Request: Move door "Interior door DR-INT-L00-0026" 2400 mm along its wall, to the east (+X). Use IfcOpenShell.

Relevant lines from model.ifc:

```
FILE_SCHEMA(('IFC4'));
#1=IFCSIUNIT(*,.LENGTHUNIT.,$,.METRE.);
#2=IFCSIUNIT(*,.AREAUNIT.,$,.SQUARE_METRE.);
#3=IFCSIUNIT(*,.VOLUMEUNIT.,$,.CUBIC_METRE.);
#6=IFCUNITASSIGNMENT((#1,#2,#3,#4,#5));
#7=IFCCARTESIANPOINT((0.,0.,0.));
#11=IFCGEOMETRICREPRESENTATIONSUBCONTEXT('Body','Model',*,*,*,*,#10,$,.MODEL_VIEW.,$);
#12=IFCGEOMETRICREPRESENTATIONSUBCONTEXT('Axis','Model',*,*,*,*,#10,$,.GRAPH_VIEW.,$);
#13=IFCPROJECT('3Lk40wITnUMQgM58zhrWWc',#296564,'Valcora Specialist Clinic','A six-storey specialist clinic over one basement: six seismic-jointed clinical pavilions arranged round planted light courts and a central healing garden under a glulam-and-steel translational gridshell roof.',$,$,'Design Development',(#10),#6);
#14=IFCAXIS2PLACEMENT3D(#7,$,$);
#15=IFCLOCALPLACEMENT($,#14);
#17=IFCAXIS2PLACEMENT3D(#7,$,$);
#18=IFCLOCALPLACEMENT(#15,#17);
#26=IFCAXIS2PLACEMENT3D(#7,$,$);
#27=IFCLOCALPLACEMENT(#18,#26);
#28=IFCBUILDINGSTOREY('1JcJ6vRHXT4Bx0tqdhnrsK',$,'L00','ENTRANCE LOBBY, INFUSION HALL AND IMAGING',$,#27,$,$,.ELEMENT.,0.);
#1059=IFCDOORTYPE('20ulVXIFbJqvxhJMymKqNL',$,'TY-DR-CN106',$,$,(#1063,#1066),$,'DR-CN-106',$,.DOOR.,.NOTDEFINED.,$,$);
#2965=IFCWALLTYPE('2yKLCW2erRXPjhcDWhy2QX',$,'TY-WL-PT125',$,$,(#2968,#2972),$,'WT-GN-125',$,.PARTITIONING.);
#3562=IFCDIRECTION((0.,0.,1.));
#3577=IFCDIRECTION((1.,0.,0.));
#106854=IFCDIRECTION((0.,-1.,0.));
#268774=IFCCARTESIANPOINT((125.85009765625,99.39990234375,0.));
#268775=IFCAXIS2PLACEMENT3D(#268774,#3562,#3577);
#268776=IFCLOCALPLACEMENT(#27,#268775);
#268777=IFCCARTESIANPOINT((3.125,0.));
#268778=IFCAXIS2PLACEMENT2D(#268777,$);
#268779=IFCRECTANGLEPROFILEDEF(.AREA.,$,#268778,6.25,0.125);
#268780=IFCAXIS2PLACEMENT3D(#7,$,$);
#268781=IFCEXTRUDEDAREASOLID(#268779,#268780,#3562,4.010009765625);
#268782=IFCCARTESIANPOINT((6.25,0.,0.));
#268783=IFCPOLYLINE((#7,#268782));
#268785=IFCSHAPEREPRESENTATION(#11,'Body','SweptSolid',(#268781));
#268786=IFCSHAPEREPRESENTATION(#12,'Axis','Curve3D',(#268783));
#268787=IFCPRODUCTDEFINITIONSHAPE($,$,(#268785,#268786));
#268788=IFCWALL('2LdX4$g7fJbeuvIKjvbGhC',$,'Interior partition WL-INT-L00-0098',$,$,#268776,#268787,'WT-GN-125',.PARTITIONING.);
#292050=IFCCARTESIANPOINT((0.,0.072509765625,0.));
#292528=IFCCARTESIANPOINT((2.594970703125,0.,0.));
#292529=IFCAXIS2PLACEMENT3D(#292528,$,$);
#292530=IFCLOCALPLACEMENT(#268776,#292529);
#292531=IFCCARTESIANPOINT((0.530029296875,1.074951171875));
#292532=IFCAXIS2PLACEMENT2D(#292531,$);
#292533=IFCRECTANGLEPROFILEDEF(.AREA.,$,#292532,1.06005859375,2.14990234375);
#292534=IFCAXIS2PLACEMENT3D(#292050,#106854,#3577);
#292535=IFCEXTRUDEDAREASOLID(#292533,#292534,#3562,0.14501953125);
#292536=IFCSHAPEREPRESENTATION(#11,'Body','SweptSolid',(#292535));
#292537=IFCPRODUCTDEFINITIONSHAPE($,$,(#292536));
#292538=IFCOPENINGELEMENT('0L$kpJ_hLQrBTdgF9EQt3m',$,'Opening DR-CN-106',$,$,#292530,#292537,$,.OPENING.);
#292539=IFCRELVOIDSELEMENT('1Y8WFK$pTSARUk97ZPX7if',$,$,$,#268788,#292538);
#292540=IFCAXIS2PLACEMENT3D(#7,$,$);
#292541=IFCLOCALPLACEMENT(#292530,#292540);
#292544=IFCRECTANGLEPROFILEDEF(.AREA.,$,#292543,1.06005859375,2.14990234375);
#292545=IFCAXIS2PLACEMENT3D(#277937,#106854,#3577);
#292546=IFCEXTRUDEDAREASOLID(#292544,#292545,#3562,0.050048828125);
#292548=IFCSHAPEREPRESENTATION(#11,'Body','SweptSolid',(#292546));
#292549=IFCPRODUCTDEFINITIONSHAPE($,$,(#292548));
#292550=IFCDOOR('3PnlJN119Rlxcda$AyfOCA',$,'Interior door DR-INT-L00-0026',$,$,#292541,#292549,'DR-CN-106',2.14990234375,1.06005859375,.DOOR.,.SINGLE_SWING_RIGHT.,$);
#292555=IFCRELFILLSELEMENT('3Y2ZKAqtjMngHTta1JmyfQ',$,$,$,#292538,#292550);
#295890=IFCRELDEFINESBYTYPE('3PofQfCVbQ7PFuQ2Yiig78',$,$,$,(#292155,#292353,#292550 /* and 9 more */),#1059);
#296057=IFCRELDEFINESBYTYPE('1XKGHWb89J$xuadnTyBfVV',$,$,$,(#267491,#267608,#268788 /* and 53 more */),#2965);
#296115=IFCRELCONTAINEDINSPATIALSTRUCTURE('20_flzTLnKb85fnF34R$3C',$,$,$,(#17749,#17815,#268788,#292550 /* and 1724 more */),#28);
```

```python
import ifcopenshell
import ifcopenshell.api.geometry
import ifcopenshell.util.placement

model = ifcopenshell.open("model.ifc")

door = model.by_guid("3PnlJN119Rlxcda$AyfOCA")
opening = door.FillsVoids[0].RelatingOpeningElement
wall = opening.VoidsElements[0].RelatingBuildingElement

wall_matrix = ifcopenshell.util.placement.get_local_placement(wall.ObjectPlacement)
shift = wall_matrix[:3, 0] * 2.4
before = ifcopenshell.util.placement.get_local_placement(door.ObjectPlacement)[:3, 3].copy()

# The door is placed relative to its opening, so it follows when the opening moves.
matrix = ifcopenshell.util.placement.get_local_placement(opening.ObjectPlacement)
matrix[:3, 3] += shift
ifcopenshell.api.geometry.edit_object_placement(
    model, product=opening, matrix=matrix, is_si=False, should_transform_children=True
)

after = ifcopenshell.util.placement.get_local_placement(door.ObjectPlacement)[:3, 3]
print("door moved by", (after - before).round(3) + 0.0)

model.write("model_rev.ifc")
```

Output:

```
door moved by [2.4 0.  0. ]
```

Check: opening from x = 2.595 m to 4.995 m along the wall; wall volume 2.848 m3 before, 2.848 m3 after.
